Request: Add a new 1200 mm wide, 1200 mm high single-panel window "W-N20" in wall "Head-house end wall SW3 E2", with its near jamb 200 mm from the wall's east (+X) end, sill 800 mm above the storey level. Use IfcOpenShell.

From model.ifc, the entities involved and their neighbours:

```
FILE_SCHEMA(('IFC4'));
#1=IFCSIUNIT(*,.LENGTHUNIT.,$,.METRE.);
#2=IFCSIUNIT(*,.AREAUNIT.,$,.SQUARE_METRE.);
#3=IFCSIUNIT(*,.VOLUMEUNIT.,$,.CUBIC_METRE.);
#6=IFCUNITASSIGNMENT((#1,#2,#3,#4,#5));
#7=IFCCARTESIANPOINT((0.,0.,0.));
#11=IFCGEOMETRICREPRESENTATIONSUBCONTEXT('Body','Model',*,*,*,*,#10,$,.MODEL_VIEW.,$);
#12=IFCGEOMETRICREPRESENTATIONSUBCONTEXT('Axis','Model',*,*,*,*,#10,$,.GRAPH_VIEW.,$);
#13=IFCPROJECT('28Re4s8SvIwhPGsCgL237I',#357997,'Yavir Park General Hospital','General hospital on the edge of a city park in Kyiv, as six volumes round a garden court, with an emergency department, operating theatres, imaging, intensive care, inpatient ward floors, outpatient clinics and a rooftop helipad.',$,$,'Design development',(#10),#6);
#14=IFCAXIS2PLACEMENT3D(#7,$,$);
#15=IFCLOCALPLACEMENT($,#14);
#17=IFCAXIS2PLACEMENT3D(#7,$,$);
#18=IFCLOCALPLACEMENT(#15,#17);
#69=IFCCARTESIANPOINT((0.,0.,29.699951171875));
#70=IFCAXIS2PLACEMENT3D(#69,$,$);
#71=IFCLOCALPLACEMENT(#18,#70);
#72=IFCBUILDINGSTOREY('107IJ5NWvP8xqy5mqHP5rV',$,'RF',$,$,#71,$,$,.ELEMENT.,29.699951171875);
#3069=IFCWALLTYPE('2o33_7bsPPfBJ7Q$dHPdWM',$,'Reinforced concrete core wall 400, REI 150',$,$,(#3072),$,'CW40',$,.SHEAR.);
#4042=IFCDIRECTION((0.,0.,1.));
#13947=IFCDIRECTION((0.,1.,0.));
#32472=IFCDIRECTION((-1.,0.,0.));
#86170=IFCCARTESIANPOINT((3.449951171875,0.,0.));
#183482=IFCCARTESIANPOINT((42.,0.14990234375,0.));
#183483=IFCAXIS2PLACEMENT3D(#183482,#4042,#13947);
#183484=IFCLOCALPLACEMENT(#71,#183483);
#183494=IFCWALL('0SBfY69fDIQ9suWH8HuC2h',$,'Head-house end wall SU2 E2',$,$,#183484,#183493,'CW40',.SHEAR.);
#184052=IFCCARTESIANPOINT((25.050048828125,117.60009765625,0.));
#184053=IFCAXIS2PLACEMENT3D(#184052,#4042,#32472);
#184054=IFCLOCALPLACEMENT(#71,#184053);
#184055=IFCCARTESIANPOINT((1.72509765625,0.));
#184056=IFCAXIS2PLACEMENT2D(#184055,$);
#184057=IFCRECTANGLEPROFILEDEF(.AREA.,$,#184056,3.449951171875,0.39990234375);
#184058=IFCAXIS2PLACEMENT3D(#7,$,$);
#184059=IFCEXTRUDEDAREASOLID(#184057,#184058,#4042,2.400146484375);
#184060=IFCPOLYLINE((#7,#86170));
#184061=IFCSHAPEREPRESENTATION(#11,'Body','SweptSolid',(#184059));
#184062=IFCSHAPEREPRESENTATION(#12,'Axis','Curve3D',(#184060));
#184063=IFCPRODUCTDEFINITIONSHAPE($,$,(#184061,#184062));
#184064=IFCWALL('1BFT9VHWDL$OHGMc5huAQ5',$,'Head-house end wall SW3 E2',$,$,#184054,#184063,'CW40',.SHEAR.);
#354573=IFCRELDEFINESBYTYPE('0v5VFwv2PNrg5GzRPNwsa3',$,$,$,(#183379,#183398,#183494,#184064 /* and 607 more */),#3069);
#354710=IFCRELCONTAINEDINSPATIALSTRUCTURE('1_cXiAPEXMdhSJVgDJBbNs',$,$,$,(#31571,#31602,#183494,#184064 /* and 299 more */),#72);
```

```python
import numpy as np
import ifcopenshell
import ifcopenshell.api.feature
import ifcopenshell.api.geometry
import ifcopenshell.api.root
import ifcopenshell.api.spatial
import ifcopenshell.geom
import ifcopenshell.util.element
import ifcopenshell.util.placement
import ifcopenshell.util.representation
import ifcopenshell.util.shape
import ifcopenshell.util.unit

model = ifcopenshell.open("model.ifc")
unit_scale = ifcopenshell.util.unit.calculate_unit_scale(model)
settings = ifcopenshell.geom.settings()


def volume(element):
    """Net volume in cubic metres, openings subtracted."""
    shape = ifcopenshell.geom.create_shape(settings, element)
    return ifcopenshell.util.shape.get_volume(shape.geometry)


wall = model.by_id(184064)
storey = ifcopenshell.util.element.get_container(wall, ifc_class="IfcBuildingStorey")
context = ifcopenshell.util.representation.get_context(model, "Model", "Body", "MODEL_VIEW")
before = volume(wall)

width, height, from_end, sill = 1.2, 1.2, 0.2, 0.8  # metres

# The wall runs along its own X axis, and the end named is its -X end.
wall_shape = ifcopenshell.geom.create_shape(settings, wall)
x, y, z = ifcopenshell.util.shape.get_vertices(wall_shape.geometry).T
start = x.min() + from_end
face, thickness = float(y.min()), float(y.max() - y.min())
wall_matrix = ifcopenshell.util.placement.get_local_placement(wall.ObjectPlacement)
level = ifcopenshell.util.placement.get_local_placement(storey.ObjectPlacement)[2, 3]


def in_wall(x, y):
    """Placement at x, y metres in the wall's axes, at sill height."""
    matrix = wall_matrix.copy()
    matrix[:, 3] = wall_matrix @ np.array([x / unit_scale, y / unit_scale, 0.0, 1.0])
    matrix[2, 3] = level + sill / unit_scale
    return matrix


# Opening: a box that overshoots both wall faces by 50 mm.
opening = ifcopenshell.api.root.create_entity(model, ifc_class="IfcOpeningElement", predefined_type="OPENING")
box = ifcopenshell.api.geometry.add_wall_representation(
    model, context=context, length=width, height=height, thickness=thickness + 0.1
)
ifcopenshell.api.geometry.assign_representation(model, product=opening, representation=box)
ifcopenshell.api.geometry.edit_object_placement(model, product=opening, matrix=in_wall(start, face - 0.05), is_si=False)
ifcopenshell.api.feature.add_feature(model, feature=opening, element=wall)

window = ifcopenshell.api.root.create_entity(model, ifc_class="IfcWindow", name="W-N20", predefined_type="WINDOW")
window.OverallWidth, window.OverallHeight = width / unit_scale, height / unit_scale
window.PartitioningType = "SINGLE_PANEL"
body = ifcopenshell.api.geometry.add_window_representation(
    model,
    context=context,
    overall_width=window.OverallWidth,
    overall_height=window.OverallHeight,
    partition_type="SINGLE_PANEL",
)
ifcopenshell.api.geometry.assign_representation(model, product=window, representation=body)
ifcopenshell.api.spatial.assign_container(model, products=[window], relating_structure=storey)
ifcopenshell.api.feature.add_filling(model, opening=opening, element=window)

# Centre the window in the wall's thickness.
ifcopenshell.api.geometry.edit_object_placement(model, product=window, matrix=in_wall(start, face), is_si=False)
window_shape = ifcopenshell.geom.create_shape(settings, window)
depth = ifcopenshell.util.shape.get_vertices(window_shape.geometry)[:, 1]
offset = face + thickness / 2 - (depth.min() + depth.max()) / 2
ifcopenshell.api.geometry.edit_object_placement(model, product=window, matrix=in_wall(start, offset), is_si=False)

after = volume(wall)

print(f"wall volume {before:.3f} -> {after:.3f} m3")

model.write("model-out.ifc")
```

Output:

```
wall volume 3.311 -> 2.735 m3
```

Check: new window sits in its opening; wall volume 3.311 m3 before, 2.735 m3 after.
